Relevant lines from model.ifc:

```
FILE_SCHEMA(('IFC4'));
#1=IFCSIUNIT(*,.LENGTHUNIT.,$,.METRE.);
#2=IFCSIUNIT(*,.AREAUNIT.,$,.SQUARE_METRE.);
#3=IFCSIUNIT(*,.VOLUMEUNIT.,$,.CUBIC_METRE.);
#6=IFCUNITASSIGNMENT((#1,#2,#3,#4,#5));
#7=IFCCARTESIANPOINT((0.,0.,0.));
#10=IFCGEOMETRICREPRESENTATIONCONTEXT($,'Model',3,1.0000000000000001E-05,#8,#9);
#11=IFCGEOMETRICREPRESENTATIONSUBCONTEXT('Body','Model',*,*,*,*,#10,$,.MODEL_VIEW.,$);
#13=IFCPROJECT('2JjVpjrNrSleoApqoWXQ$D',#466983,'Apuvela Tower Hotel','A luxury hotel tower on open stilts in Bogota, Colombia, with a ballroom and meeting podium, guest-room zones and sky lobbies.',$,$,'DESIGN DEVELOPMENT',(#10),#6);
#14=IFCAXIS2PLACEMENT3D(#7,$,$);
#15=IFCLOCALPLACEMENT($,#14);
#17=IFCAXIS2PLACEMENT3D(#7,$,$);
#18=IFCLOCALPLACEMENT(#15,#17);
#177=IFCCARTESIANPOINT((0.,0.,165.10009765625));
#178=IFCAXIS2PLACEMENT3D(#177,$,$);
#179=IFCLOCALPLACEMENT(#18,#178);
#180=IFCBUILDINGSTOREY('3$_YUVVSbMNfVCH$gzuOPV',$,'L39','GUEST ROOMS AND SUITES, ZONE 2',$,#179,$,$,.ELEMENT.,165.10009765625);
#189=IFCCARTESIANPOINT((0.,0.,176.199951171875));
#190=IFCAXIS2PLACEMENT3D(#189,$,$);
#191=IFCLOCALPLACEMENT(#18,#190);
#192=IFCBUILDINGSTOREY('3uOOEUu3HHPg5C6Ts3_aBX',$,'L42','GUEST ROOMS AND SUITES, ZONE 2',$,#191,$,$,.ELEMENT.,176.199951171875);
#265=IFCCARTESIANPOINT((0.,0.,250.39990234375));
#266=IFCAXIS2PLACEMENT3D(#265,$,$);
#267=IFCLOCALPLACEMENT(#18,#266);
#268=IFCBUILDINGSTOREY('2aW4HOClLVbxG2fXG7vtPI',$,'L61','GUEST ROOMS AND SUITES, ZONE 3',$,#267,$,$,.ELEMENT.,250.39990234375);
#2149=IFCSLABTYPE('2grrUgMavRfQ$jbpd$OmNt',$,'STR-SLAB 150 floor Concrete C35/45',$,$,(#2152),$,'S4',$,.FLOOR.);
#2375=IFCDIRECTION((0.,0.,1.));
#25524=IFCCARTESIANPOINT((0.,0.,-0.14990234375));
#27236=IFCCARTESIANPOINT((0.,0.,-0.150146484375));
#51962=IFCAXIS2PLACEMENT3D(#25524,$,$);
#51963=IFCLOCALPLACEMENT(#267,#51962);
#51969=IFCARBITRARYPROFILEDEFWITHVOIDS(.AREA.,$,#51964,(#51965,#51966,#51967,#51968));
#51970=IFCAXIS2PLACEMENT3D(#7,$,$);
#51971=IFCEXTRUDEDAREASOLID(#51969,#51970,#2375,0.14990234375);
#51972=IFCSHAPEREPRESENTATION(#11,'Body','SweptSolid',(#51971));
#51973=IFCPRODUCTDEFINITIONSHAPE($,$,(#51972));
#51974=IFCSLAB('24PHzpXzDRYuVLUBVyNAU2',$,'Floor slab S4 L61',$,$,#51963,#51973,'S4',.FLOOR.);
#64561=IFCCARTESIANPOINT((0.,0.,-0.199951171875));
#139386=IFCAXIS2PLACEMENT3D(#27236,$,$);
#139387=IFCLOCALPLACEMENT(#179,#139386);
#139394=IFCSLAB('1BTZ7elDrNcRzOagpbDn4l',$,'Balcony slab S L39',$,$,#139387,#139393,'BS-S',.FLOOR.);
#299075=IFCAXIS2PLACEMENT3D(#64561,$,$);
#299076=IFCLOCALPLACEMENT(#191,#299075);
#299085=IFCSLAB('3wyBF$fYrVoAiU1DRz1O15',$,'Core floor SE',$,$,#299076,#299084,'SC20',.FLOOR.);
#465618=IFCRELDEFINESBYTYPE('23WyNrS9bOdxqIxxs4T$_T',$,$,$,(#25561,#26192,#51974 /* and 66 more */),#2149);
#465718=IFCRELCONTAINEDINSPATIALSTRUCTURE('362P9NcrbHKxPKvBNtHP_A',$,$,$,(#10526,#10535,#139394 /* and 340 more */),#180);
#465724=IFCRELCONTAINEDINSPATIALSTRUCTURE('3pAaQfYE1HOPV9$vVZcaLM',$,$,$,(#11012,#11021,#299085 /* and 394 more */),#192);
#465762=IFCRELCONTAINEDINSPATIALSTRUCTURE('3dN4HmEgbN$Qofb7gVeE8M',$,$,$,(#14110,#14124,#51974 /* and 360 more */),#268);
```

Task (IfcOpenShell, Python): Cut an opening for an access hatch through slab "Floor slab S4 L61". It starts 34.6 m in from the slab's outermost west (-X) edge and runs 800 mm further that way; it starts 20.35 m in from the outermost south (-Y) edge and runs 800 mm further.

```python
import numpy as np
import ifcopenshell
import ifcopenshell.api.feature
import ifcopenshell.api.geometry
import ifcopenshell.api.root
import ifcopenshell.geom
import ifcopenshell.util.placement
import ifcopenshell.util.representation
import ifcopenshell.util.shape
import ifcopenshell.util.unit

model = ifcopenshell.open("model.ifc")
unit_scale = ifcopenshell.util.unit.calculate_unit_scale(model)
settings = ifcopenshell.geom.settings()


def volume(element):
    """Net volume in cubic metres, openings subtracted."""
    shape = ifcopenshell.geom.create_shape(settings, element)
    return ifcopenshell.util.shape.get_volume(shape.geometry)


slab = model.by_id(51974)
before = volume(slab)

# Extent in the slab's own axes, in metres. The edges named are its -X and -Y sides.
slab_shape = ifcopenshell.geom.create_shape(settings, slab)
vertices = ifcopenshell.util.shape.get_vertices(slab_shape.geometry)
x_min, y_min, bottom = vertices.min(axis=0)
top = vertices[:, 2].max()

opening = ifcopenshell.api.root.create_entity(model, ifc_class="IfcOpeningElement", name="Access hatch opening", predefined_type="OPENING")
context = ifcopenshell.util.representation.get_context(model, "Model", "Body", "MODEL_VIEW")
width, depth = 0.8, 0.8
outline = [(0.0, 0.0), (width, 0.0), (width, depth), (0.0, depth), (0.0, 0.0)]
# Overshoot both faces by 50 mm so the cut is clean.
shape = ifcopenshell.api.geometry.add_slab_representation(
    model, context=context, depth=top - bottom + 0.1, polyline=outline
)
ifcopenshell.api.geometry.assign_representation(model, product=opening, representation=shape)

matrix = ifcopenshell.util.placement.get_local_placement(slab.ObjectPlacement)
matrix[:, 3] = matrix @ np.append(np.array([x_min + 34.6, y_min + 20.35, bottom - 0.05]) / unit_scale, 1.0)
ifcopenshell.api.geometry.edit_object_placement(model, product=opening, matrix=matrix, is_si=False)
ifcopenshell.api.feature.add_feature(model, feature=opening, element=slab)

after = volume(slab)

print(f"slab volume {before:.3f} -> {after:.3f} m3")

model.write("model_edited.ifc")
```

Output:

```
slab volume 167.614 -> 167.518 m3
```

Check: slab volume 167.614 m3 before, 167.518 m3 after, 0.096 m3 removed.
